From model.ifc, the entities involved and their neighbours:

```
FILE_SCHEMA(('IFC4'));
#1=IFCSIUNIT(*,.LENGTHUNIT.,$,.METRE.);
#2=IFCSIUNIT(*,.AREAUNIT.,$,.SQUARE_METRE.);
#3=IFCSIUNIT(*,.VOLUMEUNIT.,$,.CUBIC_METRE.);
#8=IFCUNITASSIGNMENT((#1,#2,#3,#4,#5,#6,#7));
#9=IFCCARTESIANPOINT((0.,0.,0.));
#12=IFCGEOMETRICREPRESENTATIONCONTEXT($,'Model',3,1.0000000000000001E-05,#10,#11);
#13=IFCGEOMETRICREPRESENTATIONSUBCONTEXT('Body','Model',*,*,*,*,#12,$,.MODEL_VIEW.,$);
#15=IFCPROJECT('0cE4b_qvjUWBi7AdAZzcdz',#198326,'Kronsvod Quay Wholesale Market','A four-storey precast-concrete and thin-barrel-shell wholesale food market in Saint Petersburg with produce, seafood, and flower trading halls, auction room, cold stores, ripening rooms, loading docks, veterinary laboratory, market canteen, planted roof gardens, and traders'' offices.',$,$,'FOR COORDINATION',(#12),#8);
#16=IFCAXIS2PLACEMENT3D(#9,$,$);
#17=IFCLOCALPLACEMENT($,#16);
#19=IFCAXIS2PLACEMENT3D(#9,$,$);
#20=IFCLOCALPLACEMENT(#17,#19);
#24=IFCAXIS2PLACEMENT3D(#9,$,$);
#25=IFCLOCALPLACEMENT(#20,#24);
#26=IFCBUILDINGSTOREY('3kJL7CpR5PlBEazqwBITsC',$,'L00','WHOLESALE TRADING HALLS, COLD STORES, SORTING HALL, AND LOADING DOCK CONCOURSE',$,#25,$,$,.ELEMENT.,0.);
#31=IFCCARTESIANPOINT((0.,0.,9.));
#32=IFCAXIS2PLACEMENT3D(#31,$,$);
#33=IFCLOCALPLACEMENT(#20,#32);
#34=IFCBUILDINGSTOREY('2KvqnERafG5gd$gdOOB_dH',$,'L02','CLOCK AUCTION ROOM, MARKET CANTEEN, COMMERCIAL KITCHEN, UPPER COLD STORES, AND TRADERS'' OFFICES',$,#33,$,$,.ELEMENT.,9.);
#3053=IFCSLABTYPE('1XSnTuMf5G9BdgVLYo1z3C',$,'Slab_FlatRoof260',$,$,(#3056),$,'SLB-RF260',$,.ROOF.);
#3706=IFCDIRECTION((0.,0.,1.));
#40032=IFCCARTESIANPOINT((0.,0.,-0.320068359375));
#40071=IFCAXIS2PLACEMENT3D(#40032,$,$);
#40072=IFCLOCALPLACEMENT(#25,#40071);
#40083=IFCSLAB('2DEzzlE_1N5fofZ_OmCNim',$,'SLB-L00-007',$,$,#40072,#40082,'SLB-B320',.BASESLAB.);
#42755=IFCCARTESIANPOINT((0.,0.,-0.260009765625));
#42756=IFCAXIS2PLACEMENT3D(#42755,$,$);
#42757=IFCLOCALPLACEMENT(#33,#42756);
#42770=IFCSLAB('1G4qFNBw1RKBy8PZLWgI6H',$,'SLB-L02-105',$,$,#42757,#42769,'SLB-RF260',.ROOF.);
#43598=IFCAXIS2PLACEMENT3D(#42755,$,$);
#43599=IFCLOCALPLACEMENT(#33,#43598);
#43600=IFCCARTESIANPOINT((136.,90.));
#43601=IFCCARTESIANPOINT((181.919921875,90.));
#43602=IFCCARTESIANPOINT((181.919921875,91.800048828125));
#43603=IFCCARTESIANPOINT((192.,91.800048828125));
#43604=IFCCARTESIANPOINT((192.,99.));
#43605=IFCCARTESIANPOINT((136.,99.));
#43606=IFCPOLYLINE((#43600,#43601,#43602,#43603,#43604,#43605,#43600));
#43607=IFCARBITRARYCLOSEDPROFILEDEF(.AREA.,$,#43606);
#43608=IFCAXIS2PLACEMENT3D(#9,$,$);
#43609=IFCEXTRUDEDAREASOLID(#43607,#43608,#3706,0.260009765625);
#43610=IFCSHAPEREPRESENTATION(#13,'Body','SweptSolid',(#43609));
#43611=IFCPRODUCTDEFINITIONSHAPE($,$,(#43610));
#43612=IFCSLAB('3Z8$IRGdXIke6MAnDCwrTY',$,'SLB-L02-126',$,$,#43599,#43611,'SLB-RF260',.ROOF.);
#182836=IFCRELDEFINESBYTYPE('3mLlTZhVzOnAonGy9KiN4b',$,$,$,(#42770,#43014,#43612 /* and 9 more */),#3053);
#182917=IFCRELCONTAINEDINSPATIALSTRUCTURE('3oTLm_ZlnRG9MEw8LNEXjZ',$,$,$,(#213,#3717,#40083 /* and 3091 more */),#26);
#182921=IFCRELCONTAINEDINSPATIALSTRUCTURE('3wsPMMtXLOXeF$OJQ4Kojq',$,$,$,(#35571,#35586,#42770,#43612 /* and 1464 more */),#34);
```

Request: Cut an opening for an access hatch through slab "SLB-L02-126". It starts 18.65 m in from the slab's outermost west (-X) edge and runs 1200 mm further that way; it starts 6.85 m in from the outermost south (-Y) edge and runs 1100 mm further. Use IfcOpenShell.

```python
import numpy as np
import ifcopenshell
import ifcopenshell.api.feature
import ifcopenshell.api.geometry
import ifcopenshell.api.root
import ifcopenshell.geom
import ifcopenshell.util.placement
import ifcopenshell.util.representation
import ifcopenshell.util.shape
import ifcopenshell.util.unit

model = ifcopenshell.open("model.ifc")
unit_scale = ifcopenshell.util.unit.calculate_unit_scale(model)
settings = ifcopenshell.geom.settings()


def volume(element):
    """Net volume in cubic metres, openings subtracted."""
    shape = ifcopenshell.geom.create_shape(settings, element)
    return ifcopenshell.util.shape.get_volume(shape.geometry)


slab = model.by_guid("3Z8$IRGdXIke6MAnDCwrTY")
before = volume(slab)

# Extent in the slab's own axes, in metres. The edges named are its -X and -Y sides.
slab_shape = ifcopenshell.geom.create_shape(settings, slab)
vertices = ifcopenshell.util.shape.get_vertices(slab_shape.geometry)
x_min, y_min, bottom = vertices.min(axis=0)
top = vertices[:, 2].max()

opening = ifcopenshell.api.root.create_entity(model, ifc_class="IfcOpeningElement", name="Access hatch opening", predefined_type="OPENING")
context = ifcopenshell.util.representation.get_context(model, "Model", "Body", "MODEL_VIEW")
width, depth = 1.2, 1.1
outline = [(0.0, 0.0), (width, 0.0), (width, depth), (0.0, depth), (0.0, 0.0)]
# Overshoot both faces by 50 mm so the cut is clean.
shape = ifcopenshell.api.geometry.add_slab_representation(
    model, context=context, depth=top - bottom + 0.1, polyline=outline
)
ifcopenshell.api.geometry.assign_representation(model, product=opening, representation=shape)

matrix = ifcopenshell.util.placement.get_local_placement(slab.ObjectPlacement)
matrix[:, 3] = matrix @ np.append(np.array([x_min + 18.65, y_min + 6.85, bottom - 0.05]) / unit_scale, 1.0)
ifcopenshell.api.geometry.edit_object_placement(model, product=opening, matrix=matrix, is_si=False)
ifcopenshell.api.feature.add_feature(model, feature=opening, element=slab)

after = volume(slab)

print(f"slab volume {before:.3f} -> {after:.3f} m3")

model.write("model_edited.ifc")
```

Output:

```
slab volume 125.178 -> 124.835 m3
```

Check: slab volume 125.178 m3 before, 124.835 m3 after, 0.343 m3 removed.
